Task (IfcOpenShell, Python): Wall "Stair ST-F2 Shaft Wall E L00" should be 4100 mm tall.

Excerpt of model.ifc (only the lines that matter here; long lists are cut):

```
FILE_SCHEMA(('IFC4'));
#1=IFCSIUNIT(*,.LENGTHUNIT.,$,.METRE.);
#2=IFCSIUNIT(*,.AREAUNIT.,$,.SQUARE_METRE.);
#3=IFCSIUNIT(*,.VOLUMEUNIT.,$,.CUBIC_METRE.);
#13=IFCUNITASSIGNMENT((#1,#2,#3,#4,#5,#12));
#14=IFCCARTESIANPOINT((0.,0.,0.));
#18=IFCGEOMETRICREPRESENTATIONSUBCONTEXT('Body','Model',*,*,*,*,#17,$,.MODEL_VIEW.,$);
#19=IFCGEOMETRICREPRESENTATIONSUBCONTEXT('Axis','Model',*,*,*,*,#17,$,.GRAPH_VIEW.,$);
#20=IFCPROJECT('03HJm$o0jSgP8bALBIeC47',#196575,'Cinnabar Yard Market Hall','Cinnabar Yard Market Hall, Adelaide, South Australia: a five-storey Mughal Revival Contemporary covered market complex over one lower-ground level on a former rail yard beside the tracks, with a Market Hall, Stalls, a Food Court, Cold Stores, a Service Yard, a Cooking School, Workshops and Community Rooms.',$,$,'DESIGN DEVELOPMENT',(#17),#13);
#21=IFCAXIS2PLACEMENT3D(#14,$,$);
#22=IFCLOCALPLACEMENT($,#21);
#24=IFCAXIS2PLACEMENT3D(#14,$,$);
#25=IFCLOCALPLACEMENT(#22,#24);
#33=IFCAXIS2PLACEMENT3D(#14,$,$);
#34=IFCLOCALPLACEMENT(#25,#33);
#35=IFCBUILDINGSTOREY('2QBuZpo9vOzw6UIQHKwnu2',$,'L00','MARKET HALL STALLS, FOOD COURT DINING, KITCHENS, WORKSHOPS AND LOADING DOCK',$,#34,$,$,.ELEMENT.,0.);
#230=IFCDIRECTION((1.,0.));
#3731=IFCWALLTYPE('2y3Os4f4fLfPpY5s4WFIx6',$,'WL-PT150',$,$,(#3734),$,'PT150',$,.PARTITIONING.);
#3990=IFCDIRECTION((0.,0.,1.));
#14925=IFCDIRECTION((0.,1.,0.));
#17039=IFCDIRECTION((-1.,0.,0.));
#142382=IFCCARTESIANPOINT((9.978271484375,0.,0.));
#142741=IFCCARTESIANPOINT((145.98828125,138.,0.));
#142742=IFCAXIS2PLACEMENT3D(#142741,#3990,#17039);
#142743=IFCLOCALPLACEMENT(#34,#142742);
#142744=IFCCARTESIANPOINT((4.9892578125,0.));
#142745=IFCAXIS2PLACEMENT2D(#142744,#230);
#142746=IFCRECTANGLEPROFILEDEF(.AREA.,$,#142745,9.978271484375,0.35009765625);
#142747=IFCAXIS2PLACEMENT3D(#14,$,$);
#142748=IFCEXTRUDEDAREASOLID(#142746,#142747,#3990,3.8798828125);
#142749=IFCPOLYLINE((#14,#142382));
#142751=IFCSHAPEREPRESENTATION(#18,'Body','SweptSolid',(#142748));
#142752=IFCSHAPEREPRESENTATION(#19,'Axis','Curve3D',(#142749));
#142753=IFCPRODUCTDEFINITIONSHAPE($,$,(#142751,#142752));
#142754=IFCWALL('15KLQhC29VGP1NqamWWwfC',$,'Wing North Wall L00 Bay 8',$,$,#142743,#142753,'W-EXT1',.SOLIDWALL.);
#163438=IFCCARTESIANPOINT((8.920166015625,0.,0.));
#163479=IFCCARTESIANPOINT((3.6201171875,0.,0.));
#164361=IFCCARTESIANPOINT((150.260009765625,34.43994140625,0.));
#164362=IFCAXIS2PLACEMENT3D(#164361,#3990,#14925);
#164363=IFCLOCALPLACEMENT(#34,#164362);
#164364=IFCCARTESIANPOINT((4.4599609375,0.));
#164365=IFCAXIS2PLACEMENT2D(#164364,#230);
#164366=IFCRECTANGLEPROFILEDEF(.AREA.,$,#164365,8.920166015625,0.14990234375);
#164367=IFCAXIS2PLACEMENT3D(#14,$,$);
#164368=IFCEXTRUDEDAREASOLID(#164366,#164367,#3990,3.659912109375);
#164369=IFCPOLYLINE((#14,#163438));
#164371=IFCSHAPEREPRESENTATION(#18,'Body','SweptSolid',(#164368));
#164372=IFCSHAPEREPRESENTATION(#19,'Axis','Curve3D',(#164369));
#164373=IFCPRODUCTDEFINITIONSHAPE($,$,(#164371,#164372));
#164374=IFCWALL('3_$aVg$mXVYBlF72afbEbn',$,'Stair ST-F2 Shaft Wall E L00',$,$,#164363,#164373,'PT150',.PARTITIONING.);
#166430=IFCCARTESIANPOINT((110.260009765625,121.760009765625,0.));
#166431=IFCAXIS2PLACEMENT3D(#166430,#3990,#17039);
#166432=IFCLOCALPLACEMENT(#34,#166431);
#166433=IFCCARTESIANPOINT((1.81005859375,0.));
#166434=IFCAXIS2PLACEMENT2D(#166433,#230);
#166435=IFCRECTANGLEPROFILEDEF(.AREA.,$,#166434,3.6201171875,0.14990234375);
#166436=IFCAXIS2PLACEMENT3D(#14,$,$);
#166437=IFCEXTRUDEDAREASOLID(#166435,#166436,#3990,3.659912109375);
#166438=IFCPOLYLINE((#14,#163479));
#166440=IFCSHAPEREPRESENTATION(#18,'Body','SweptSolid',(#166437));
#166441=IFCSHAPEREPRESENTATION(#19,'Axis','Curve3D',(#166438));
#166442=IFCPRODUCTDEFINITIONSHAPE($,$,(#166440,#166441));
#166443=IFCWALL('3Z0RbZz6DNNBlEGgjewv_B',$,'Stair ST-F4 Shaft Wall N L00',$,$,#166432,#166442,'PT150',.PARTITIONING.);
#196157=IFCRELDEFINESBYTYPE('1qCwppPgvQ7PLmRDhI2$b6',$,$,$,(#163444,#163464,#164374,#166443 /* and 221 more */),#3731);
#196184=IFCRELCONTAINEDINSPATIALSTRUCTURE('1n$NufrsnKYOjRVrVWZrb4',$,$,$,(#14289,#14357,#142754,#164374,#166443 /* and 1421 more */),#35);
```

```python
import ifcopenshell
import ifcopenshell.geom
import ifcopenshell.util.representation
import ifcopenshell.util.shape

model = ifcopenshell.open("model.ifc")
settings = ifcopenshell.geom.settings()


def volume(element):
    """Net volume in cubic metres, openings subtracted."""
    shape = ifcopenshell.geom.create_shape(settings, element)
    return ifcopenshell.util.shape.get_volume(shape.geometry)


wall = model.by_guid("3_$aVg$mXVYBlF72afbEbn")
before = volume(wall)

body = ifcopenshell.util.representation.get_representation(wall, "Model", "Body")
solid = body.Items[0]
old_height = solid.Depth
solid.Depth = 4.1
after = volume(wall)

print(f"height {old_height:g} -> {solid.Depth:g}, volume {before:.3f} -> {after:.3f} m3")

model.write("model_rev.ifc")
```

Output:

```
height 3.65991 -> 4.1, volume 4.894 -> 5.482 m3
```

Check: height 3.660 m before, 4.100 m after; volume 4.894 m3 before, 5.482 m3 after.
